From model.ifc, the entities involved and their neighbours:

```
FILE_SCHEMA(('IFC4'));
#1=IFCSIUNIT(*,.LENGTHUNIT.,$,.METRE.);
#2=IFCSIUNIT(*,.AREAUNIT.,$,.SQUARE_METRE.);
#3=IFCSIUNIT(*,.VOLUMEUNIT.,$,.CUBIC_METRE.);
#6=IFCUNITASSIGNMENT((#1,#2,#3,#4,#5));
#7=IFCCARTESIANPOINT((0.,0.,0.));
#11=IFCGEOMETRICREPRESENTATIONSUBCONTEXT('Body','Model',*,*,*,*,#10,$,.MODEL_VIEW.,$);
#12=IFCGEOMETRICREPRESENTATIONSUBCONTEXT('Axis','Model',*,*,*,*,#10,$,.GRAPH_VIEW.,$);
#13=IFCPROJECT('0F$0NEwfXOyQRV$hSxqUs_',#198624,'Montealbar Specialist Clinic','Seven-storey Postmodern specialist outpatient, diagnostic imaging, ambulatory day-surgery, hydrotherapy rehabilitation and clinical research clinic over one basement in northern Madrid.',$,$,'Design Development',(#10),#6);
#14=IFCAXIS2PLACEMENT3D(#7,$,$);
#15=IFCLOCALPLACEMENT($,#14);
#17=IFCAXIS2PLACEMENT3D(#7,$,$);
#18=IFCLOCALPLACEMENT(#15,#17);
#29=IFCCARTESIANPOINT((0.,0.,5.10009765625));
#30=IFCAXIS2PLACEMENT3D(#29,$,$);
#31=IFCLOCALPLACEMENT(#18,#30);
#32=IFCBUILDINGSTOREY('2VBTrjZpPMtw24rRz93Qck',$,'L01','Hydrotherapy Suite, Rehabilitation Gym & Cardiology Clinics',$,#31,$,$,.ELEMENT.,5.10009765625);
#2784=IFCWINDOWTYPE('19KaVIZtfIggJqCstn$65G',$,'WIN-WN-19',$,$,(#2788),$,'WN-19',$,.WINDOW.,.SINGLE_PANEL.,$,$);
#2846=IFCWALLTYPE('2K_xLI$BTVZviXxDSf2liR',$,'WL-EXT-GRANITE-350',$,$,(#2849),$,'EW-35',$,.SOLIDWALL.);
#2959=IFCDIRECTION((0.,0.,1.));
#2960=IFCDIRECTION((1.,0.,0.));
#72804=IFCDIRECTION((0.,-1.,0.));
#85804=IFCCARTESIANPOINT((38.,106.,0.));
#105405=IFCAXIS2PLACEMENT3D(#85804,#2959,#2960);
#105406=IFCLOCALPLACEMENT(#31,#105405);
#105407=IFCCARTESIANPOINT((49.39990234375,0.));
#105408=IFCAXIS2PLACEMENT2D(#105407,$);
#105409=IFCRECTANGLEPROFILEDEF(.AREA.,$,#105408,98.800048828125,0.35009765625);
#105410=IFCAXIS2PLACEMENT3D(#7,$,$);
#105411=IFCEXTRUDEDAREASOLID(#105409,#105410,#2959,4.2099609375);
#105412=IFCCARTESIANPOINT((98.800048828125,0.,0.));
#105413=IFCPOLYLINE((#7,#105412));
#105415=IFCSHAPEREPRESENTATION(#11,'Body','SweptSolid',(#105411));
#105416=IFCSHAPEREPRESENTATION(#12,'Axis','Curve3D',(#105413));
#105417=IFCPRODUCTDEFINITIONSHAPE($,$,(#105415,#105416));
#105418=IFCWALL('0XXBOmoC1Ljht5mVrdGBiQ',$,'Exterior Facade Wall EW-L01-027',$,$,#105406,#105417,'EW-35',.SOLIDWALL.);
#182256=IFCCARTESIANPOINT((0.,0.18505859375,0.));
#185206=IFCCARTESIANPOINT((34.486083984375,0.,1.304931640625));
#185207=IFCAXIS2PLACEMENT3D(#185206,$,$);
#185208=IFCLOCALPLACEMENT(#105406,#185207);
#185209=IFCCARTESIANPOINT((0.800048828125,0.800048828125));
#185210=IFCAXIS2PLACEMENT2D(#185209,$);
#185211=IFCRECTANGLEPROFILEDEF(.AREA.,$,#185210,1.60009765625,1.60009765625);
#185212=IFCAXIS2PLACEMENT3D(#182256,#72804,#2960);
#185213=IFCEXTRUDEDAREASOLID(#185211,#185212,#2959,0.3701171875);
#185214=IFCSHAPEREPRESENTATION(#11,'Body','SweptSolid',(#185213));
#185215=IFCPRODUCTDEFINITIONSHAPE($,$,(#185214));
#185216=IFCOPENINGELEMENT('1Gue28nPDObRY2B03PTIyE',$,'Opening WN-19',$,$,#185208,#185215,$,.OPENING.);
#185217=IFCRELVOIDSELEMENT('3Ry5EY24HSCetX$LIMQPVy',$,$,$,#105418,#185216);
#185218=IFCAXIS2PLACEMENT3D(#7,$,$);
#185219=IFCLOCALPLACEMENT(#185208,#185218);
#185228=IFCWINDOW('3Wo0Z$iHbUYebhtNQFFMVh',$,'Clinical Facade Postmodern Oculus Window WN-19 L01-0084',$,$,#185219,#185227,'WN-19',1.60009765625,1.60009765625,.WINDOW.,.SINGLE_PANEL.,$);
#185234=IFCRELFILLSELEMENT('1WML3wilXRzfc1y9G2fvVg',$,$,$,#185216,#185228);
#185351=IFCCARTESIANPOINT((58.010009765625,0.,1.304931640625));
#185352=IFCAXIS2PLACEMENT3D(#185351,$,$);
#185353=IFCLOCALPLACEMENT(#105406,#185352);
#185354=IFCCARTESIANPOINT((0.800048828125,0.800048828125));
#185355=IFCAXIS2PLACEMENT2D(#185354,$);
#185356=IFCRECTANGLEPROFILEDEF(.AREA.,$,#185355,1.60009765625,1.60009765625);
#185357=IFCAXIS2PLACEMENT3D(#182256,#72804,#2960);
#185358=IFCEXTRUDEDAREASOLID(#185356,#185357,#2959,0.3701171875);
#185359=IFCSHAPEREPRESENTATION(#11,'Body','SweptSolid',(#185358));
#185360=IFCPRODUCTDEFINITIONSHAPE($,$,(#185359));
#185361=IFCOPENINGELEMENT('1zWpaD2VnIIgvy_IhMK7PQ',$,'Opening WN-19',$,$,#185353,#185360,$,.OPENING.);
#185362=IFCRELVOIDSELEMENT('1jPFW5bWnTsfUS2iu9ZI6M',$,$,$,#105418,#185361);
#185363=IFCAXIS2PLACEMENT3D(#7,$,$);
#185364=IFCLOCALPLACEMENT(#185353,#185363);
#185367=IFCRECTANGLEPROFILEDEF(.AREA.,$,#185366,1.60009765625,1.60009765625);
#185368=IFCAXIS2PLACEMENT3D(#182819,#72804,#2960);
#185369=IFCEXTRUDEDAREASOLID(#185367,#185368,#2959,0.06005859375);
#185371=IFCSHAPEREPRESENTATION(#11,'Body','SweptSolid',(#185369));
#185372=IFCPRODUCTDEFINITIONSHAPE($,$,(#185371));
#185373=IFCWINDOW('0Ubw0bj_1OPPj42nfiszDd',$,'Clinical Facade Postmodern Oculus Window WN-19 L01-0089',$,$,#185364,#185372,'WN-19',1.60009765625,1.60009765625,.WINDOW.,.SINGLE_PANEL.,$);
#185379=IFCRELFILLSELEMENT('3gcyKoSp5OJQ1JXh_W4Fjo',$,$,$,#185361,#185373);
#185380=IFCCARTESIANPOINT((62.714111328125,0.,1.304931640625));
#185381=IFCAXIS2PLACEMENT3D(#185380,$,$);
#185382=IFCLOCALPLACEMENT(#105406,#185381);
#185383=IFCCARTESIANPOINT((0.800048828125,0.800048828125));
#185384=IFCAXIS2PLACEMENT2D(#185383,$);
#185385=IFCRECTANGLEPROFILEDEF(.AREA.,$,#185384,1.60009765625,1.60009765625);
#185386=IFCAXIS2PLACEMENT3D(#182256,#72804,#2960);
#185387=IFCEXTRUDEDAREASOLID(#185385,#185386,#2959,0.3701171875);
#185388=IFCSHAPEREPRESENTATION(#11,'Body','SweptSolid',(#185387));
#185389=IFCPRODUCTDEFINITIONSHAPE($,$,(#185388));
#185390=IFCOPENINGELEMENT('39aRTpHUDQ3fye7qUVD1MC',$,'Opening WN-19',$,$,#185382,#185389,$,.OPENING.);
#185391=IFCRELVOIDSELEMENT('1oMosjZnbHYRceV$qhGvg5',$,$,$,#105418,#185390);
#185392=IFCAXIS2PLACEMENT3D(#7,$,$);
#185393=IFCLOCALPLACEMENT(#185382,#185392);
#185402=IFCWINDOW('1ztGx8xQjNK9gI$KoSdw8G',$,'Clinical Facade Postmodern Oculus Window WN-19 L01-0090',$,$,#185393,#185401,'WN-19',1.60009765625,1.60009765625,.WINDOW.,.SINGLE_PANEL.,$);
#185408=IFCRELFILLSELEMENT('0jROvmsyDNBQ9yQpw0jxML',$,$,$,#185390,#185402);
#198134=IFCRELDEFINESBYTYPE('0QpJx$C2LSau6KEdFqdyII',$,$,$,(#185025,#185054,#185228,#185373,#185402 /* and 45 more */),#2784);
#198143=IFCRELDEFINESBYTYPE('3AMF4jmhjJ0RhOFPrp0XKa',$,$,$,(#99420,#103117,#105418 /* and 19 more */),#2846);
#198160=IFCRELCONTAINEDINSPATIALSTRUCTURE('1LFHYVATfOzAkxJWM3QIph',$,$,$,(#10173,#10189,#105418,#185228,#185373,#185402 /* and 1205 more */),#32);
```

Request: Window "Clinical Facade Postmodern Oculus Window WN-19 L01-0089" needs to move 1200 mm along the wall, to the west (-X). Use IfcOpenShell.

```python
import ifcopenshell
import ifcopenshell.api.geometry
import ifcopenshell.util.placement
import ifcopenshell.util.unit

model = ifcopenshell.open("model.ifc")
unit_scale = ifcopenshell.util.unit.calculate_unit_scale(model)

window = model.by_guid("0Ubw0bj_1OPPj42nfiszDd")
opening = window.FillsVoids[0].RelatingOpeningElement
wall = opening.VoidsElements[0].RelatingBuildingElement

wall_matrix = ifcopenshell.util.placement.get_local_placement(wall.ObjectPlacement)
shift = wall_matrix[:3, 0] * -1.2 / unit_scale
before = ifcopenshell.util.placement.get_local_placement(window.ObjectPlacement)[:3, 3].copy()

# The window is placed relative to its opening, so it follows when the opening moves.
matrix = ifcopenshell.util.placement.get_local_placement(opening.ObjectPlacement)
matrix[:3, 3] += shift
ifcopenshell.api.geometry.edit_object_placement(
    model, product=opening, matrix=matrix, is_si=False, should_transform_children=True
)

after = ifcopenshell.util.placement.get_local_placement(window.ObjectPlacement)[:3, 3]
print("window moved by", (after - before).round(3) + 0.0)

model.write("model_updated.ifc")
```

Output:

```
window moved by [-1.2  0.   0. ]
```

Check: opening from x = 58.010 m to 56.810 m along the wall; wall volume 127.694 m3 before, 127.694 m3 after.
